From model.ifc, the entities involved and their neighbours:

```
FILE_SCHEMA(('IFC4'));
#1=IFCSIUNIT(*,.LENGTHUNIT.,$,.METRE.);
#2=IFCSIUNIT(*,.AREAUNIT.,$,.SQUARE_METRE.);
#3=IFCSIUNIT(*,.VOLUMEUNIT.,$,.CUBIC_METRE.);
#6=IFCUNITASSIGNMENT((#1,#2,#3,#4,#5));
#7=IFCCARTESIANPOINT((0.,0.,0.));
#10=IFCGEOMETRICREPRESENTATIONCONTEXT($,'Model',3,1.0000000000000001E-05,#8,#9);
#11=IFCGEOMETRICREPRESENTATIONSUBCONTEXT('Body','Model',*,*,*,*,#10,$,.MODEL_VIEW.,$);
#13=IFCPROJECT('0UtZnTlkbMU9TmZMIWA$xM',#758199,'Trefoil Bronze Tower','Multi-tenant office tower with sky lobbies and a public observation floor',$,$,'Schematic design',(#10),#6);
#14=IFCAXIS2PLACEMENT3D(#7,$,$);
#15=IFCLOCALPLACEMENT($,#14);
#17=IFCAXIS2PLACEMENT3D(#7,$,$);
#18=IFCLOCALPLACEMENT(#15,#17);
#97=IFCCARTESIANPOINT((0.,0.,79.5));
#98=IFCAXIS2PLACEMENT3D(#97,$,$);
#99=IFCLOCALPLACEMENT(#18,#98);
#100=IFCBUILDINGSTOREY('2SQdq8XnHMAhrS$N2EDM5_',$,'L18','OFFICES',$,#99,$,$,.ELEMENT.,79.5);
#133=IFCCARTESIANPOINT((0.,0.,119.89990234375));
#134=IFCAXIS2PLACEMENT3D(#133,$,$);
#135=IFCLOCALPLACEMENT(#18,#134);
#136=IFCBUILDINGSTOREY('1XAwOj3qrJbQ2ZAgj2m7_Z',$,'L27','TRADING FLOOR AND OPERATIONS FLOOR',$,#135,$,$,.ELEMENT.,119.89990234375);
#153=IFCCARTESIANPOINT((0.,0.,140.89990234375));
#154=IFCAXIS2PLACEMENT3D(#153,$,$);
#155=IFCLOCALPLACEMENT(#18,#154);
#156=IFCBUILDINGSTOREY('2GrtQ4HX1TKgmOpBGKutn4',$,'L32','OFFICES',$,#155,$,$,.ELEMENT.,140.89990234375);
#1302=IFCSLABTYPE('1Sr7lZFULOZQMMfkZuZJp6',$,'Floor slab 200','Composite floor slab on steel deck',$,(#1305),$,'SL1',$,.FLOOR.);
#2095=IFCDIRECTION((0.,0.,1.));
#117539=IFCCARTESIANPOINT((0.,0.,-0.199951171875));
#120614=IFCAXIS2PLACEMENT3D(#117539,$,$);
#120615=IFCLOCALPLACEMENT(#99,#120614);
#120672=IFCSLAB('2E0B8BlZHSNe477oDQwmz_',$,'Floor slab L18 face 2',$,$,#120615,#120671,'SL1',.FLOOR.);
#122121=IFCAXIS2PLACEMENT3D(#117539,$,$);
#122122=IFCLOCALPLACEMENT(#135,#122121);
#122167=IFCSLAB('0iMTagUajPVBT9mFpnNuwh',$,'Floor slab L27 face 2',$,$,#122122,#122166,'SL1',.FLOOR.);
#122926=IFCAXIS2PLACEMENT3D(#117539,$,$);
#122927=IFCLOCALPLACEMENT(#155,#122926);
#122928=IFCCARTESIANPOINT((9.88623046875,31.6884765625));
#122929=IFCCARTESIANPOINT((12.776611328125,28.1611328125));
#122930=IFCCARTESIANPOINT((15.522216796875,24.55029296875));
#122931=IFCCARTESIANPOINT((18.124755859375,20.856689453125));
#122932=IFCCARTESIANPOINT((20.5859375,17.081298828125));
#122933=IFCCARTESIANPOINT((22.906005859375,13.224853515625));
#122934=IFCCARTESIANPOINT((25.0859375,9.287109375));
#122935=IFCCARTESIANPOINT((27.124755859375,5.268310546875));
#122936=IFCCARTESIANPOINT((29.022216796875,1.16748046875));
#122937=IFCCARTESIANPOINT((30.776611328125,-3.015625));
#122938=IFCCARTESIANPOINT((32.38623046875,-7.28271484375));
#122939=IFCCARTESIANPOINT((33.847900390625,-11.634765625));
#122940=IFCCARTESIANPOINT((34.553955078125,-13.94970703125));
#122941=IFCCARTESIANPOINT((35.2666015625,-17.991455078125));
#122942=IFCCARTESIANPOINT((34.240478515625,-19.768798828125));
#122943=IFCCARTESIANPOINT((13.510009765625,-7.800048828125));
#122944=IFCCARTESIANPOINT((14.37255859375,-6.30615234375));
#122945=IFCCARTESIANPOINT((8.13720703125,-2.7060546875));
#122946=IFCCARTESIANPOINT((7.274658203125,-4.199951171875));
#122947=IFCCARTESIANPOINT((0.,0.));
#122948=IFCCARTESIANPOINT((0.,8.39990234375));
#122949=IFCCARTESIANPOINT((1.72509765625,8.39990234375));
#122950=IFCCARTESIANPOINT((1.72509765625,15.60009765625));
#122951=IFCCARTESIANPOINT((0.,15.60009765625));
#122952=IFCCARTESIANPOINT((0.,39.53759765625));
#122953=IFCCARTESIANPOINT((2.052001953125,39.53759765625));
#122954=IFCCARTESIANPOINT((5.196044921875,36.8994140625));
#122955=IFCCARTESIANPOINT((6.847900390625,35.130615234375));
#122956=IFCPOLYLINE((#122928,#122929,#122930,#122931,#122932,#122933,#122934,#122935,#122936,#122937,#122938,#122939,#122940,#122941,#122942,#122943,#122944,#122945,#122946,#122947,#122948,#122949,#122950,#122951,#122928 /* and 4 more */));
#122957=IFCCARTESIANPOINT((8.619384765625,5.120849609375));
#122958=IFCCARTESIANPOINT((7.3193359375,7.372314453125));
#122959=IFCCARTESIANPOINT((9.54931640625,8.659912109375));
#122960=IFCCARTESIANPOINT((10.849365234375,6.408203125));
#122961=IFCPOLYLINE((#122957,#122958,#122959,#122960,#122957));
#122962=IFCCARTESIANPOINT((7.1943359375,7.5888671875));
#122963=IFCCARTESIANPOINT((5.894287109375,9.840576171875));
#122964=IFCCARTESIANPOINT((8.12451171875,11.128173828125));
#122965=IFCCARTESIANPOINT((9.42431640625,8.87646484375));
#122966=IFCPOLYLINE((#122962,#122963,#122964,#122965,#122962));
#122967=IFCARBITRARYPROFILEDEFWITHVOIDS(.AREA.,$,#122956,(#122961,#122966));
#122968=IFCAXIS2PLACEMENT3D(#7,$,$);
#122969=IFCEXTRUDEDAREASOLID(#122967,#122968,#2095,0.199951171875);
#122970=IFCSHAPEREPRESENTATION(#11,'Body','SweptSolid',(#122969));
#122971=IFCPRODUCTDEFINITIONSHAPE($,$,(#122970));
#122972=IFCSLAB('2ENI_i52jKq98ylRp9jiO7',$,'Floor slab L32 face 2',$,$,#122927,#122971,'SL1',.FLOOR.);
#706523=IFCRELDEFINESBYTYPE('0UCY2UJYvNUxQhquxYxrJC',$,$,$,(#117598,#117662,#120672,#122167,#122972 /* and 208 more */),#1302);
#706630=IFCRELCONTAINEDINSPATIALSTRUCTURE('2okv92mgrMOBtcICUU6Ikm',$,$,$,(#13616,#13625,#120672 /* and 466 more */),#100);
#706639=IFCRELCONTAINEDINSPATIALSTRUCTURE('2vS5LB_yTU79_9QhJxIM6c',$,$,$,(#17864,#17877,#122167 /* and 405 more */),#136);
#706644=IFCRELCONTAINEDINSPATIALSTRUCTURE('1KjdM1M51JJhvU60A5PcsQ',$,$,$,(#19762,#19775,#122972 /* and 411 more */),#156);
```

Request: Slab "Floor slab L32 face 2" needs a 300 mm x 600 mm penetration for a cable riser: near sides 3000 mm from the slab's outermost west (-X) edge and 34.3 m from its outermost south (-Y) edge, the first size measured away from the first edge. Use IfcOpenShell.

```python
import numpy as np
import ifcopenshell
import ifcopenshell.api.feature
import ifcopenshell.api.geometry
import ifcopenshell.api.root
import ifcopenshell.geom
import ifcopenshell.util.placement
import ifcopenshell.util.representation
import ifcopenshell.util.shape
import ifcopenshell.util.unit

model = ifcopenshell.open("model.ifc")
unit_scale = ifcopenshell.util.unit.calculate_unit_scale(model)
settings = ifcopenshell.geom.settings()


def volume(element):
    """Net volume in cubic metres, openings subtracted."""
    shape = ifcopenshell.geom.create_shape(settings, element)
    return ifcopenshell.util.shape.get_volume(shape.geometry)


slab = model.by_guid("2ENI_i52jKq98ylRp9jiO7")
before = volume(slab)

# Extent in the slab's own axes, in metres. The edges named are its -X and -Y sides.
slab_shape = ifcopenshell.geom.create_shape(settings, slab)
vertices = ifcopenshell.util.shape.get_vertices(slab_shape.geometry)
x_min, y_min, bottom = vertices.min(axis=0)
top = vertices[:, 2].max()

opening = ifcopenshell.api.root.create_entity(model, ifc_class="IfcOpeningElement", name="Cable riser opening", predefined_type="OPENING")
context = ifcopenshell.util.representation.get_context(model, "Model", "Body", "MODEL_VIEW")
width, depth = 0.3, 0.6
outline = [(0.0, 0.0), (width, 0.0), (width, depth), (0.0, depth), (0.0, 0.0)]
# Overshoot both faces by 50 mm so the cut is clean.
shape = ifcopenshell.api.geometry.add_slab_representation(
    model, context=context, depth=top - bottom + 0.1, polyline=outline
)
ifcopenshell.api.geometry.assign_representation(model, product=opening, representation=shape)

matrix = ifcopenshell.util.placement.get_local_placement(slab.ObjectPlacement)
matrix[:, 3] = matrix @ np.append(np.array([x_min + 3, y_min + 34.3, bottom - 0.05]) / unit_scale, 1.0)
ifcopenshell.api.geometry.edit_object_placement(model, product=opening, matrix=matrix, is_si=False)
ifcopenshell.api.feature.add_feature(model, feature=opening, element=slab)

after = volume(slab)

print(f"slab volume {before:.3f} -> {after:.3f} m3")

model.write("model_updated.ifc")
```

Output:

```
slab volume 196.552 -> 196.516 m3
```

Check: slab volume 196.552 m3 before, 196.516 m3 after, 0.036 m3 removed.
